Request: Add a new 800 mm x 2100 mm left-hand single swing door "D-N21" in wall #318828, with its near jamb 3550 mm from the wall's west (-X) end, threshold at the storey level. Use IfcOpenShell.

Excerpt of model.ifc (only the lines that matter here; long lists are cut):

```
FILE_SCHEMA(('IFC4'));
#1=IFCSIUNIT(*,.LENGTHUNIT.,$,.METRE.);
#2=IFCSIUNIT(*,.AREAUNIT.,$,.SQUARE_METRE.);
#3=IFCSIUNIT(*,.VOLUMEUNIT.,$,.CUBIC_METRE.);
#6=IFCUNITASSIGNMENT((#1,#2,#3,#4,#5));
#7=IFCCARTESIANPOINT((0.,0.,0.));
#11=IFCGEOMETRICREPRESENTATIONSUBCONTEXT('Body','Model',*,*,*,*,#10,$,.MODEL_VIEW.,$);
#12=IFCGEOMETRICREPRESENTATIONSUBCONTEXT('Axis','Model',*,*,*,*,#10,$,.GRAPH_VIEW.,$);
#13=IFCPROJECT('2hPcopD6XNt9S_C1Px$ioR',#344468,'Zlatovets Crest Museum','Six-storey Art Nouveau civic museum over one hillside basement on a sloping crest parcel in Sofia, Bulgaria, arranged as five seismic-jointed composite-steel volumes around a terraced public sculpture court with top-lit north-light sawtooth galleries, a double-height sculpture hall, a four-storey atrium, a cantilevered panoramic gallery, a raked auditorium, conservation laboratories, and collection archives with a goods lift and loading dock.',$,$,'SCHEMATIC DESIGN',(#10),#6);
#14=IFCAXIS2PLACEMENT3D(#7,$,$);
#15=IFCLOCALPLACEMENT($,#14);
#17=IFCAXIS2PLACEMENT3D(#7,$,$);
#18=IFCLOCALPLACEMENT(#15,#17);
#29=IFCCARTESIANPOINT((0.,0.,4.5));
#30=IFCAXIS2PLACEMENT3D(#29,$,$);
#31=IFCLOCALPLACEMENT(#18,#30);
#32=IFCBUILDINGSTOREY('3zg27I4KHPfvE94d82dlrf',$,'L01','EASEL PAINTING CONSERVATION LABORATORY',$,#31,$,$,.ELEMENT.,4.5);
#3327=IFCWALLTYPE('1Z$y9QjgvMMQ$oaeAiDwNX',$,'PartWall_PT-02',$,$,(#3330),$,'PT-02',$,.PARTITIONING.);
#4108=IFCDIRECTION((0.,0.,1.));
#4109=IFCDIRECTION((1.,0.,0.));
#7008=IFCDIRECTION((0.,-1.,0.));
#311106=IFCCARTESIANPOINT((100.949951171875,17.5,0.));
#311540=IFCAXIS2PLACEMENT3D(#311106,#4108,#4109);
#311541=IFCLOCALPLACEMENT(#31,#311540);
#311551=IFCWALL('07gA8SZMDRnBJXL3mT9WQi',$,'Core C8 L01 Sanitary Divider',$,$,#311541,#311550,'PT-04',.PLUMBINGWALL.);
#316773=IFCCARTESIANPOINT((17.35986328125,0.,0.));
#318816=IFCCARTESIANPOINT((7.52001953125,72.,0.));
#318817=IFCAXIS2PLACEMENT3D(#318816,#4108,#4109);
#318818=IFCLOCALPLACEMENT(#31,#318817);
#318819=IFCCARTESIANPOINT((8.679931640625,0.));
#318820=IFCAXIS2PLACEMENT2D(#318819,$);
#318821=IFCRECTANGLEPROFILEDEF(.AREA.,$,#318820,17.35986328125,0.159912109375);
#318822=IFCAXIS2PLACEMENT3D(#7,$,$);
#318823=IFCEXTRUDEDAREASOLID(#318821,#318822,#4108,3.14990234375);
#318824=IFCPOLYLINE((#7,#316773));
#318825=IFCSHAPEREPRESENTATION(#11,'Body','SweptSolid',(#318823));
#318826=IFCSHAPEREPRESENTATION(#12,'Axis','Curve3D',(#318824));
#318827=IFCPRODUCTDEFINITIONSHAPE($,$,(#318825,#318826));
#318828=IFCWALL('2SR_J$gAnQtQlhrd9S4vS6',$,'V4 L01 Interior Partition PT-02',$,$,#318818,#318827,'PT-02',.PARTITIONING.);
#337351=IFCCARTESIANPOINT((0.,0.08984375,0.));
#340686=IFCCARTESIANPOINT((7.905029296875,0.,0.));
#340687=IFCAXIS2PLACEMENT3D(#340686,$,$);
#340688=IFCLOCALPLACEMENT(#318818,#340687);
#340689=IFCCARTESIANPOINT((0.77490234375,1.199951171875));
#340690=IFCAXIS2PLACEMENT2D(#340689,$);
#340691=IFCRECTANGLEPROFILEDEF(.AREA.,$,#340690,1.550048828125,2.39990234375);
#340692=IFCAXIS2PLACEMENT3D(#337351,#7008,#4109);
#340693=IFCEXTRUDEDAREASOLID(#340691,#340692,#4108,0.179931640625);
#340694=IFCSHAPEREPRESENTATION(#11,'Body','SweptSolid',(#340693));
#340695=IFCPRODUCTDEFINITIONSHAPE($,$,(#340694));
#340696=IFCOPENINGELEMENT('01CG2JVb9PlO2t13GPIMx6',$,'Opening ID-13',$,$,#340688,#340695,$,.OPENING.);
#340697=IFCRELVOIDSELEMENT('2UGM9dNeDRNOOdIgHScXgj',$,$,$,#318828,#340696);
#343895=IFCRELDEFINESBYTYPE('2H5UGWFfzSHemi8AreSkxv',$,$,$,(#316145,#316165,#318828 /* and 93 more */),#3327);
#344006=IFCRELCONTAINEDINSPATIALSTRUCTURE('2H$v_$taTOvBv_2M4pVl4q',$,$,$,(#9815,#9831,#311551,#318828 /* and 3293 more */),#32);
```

```python
import numpy as np
import ifcopenshell
import ifcopenshell.api.feature
import ifcopenshell.api.geometry
import ifcopenshell.api.root
import ifcopenshell.api.spatial
import ifcopenshell.geom
import ifcopenshell.util.element
import ifcopenshell.util.placement
import ifcopenshell.util.representation
import ifcopenshell.util.shape
import ifcopenshell.util.unit

model = ifcopenshell.open("model.ifc")
unit_scale = ifcopenshell.util.unit.calculate_unit_scale(model)
settings = ifcopenshell.geom.settings()


def volume(element):
    """Net volume in cubic metres, openings subtracted."""
    shape = ifcopenshell.geom.create_shape(settings, element)
    return ifcopenshell.util.shape.get_volume(shape.geometry)


wall = model.by_guid("2SR_J$gAnQtQlhrd9S4vS6")
storey = ifcopenshell.util.element.get_container(wall, ifc_class="IfcBuildingStorey")
context = ifcopenshell.util.representation.get_context(model, "Model", "Body", "MODEL_VIEW")
before = volume(wall)

width, height, from_end, sill = 0.8, 2.1, 3.55, 0.0  # metres

# The wall runs along its own X axis, and the end named is its -X end.
wall_shape = ifcopenshell.geom.create_shape(settings, wall)
x, y, z = ifcopenshell.util.shape.get_vertices(wall_shape.geometry).T
start = x.min() + from_end
face, thickness = float(y.min()), float(y.max() - y.min())
wall_matrix = ifcopenshell.util.placement.get_local_placement(wall.ObjectPlacement)
level = ifcopenshell.util.placement.get_local_placement(storey.ObjectPlacement)[2, 3]


def in_wall(x, y):
    """Placement at x, y metres in the wall's axes, at sill height."""
    matrix = wall_matrix.copy()
    matrix[:, 3] = wall_matrix @ np.array([x / unit_scale, y / unit_scale, 0.0, 1.0])
    matrix[2, 3] = level + sill / unit_scale
    return matrix


# Opening: a box that overshoots both wall faces by 50 mm.
opening = ifcopenshell.api.root.create_entity(model, ifc_class="IfcOpeningElement", predefined_type="OPENING")
box = ifcopenshell.api.geometry.add_wall_representation(
    model, context=context, length=width, height=height, thickness=thickness + 0.1
)
ifcopenshell.api.geometry.assign_representation(model, product=opening, representation=box)
ifcopenshell.api.geometry.edit_object_placement(model, product=opening, matrix=in_wall(start, face - 0.05), is_si=False)
ifcopenshell.api.feature.add_feature(model, feature=opening, element=wall)

door = ifcopenshell.api.root.create_entity(model, ifc_class="IfcDoor", name="D-N21", predefined_type="DOOR")
door.OverallWidth, door.OverallHeight = width / unit_scale, height / unit_scale
door.OperationType = "SINGLE_SWING_LEFT"
body = ifcopenshell.api.geometry.add_door_representation(
    model,
    context=context,
    overall_width=door.OverallWidth,
    overall_height=door.OverallHeight,
    operation_type="SINGLE_SWING_LEFT",
    lining_properties={"LiningDepth": thickness / unit_scale, "ThresholdDepth": thickness / unit_scale},
)
ifcopenshell.api.geometry.assign_representation(model, product=door, representation=body)
ifcopenshell.api.spatial.assign_container(model, products=[door], relating_structure=storey)
ifcopenshell.api.feature.add_filling(model, opening=opening, element=door)

# The lining spans the wall, so the door starts at the wall face.
ifcopenshell.api.geometry.edit_object_placement(model, product=door, matrix=in_wall(start, face), is_si=False)

after = volume(wall)

print(f"wall volume {before:.3f} -> {after:.3f} m3")

model.write("model_rev.ifc")
```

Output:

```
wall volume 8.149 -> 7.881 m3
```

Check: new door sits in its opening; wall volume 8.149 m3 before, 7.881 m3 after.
